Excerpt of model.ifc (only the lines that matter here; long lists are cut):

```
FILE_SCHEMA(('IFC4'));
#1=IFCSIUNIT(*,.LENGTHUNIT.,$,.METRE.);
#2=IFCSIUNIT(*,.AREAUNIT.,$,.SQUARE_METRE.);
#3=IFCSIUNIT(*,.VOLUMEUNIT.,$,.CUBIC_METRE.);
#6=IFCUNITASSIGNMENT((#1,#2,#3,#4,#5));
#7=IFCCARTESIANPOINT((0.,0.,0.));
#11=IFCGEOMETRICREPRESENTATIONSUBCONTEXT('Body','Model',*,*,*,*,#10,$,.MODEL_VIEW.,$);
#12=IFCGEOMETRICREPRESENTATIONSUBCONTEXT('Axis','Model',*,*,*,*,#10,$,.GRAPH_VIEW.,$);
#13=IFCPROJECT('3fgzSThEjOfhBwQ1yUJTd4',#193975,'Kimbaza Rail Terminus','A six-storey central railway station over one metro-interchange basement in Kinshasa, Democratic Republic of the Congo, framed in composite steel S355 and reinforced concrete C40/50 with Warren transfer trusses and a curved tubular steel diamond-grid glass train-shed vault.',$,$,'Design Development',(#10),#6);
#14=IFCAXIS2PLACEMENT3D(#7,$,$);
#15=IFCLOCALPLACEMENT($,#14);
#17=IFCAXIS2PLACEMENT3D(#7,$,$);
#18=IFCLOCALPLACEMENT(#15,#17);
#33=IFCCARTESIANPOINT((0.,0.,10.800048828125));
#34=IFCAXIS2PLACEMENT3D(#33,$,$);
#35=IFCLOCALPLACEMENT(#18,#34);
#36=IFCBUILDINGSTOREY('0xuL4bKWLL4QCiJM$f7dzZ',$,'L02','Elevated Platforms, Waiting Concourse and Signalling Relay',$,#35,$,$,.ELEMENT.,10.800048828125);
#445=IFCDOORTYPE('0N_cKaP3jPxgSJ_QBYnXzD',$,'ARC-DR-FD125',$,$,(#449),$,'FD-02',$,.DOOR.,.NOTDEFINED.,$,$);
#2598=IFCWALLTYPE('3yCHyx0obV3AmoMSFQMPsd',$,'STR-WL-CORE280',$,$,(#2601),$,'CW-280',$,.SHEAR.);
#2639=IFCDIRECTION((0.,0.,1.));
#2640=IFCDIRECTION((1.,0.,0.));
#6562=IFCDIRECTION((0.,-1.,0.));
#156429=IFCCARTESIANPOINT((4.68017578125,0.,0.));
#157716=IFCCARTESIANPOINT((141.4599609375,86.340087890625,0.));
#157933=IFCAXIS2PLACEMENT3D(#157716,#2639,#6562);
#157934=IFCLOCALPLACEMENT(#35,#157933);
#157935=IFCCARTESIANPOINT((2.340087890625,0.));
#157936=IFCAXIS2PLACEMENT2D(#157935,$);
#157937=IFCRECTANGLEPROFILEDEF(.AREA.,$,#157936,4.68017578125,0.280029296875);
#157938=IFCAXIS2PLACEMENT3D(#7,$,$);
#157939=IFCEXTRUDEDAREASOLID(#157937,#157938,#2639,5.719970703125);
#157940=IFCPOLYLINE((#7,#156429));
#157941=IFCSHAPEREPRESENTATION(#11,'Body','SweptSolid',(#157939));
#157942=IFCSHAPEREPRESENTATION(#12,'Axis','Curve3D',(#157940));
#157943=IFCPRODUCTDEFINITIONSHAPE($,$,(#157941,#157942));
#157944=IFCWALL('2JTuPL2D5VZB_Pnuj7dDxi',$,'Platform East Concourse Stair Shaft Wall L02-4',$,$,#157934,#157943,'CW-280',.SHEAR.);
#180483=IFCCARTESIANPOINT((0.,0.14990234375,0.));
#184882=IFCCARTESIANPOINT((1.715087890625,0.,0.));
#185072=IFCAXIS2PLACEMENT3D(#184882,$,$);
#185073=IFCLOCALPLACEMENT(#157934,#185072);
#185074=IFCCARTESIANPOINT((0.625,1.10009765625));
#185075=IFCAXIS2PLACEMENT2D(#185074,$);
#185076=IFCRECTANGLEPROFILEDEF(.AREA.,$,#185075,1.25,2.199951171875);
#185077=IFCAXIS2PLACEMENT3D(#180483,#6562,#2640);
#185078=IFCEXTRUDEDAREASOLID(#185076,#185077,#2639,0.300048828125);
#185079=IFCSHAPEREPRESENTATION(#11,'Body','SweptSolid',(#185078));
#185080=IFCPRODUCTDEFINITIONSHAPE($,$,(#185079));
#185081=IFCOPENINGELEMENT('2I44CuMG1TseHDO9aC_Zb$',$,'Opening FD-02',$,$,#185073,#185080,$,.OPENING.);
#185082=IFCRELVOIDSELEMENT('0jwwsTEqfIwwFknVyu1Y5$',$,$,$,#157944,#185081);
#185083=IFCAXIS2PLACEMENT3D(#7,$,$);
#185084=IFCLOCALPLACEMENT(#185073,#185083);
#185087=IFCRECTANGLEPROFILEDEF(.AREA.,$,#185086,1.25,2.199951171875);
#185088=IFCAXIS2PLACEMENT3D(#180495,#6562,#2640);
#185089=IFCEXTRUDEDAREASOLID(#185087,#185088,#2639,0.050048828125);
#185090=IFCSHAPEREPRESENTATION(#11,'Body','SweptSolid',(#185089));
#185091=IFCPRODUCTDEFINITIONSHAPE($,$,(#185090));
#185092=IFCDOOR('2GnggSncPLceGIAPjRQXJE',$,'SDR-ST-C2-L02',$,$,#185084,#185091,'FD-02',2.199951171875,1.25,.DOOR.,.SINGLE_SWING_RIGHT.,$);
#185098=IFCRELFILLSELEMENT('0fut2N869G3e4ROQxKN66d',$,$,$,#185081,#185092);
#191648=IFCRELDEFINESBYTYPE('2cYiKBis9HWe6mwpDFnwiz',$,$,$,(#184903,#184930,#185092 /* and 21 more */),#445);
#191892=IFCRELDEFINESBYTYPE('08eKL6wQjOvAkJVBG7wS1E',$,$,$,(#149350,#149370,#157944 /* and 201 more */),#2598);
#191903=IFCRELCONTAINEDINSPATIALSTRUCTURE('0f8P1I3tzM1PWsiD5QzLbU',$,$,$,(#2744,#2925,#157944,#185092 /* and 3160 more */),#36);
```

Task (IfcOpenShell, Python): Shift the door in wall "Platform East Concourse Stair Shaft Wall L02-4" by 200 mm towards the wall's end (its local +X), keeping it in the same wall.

```python
import ifcopenshell
import ifcopenshell.api.geometry
import ifcopenshell.util.placement
import ifcopenshell.util.unit

model = ifcopenshell.open("model.ifc")
unit_scale = ifcopenshell.util.unit.calculate_unit_scale(model)

door = model.by_id(185092)
opening = door.FillsVoids[0].RelatingOpeningElement
wall = opening.VoidsElements[0].RelatingBuildingElement

wall_matrix = ifcopenshell.util.placement.get_local_placement(wall.ObjectPlacement)
shift = wall_matrix[:3, 0] * 0.2 / unit_scale
before = ifcopenshell.util.placement.get_local_placement(door.ObjectPlacement)[:3, 3].copy()

# The door is placed relative to its opening, so it follows when the opening moves.
matrix = ifcopenshell.util.placement.get_local_placement(opening.ObjectPlacement)
matrix[:3, 3] += shift
ifcopenshell.api.geometry.edit_object_placement(
    model, product=opening, matrix=matrix, is_si=False, should_transform_children=True
)

after = ifcopenshell.util.placement.get_local_placement(door.ObjectPlacement)[:3, 3]
print("door moved by", (after - before).round(3) + 0.0)

model.write("model-out.ifc")
```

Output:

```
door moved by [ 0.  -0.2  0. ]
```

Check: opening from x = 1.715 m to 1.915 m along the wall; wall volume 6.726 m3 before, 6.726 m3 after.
